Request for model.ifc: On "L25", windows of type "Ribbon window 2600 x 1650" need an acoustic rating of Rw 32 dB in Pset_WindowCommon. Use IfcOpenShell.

First a look at what the model holds.

```python
import ifcopenshell
import ifcopenshell.util.element

model = ifcopenshell.open("model.ifc")
print(model.schema)
storey = next(s for s in model.by_type("IfcBuildingStorey") if s.Name == "L25")
windows = [e for e in ifcopenshell.util.element.get_decomposition(storey) if e.is_a("IfcWindow")]
seen = {}
for e in windows:
    element_type = ifcopenshell.util.element.get_type(e)
    key = (element_type.Name if element_type != e and element_type else None, ifcopenshell.util.element.get_pset(e, "Pset_WindowCommon", "AcousticRating"))
    seen[key] = seen.get(key, 0) + 1
for (name, value), count in sorted(seen.items(), key=str):
    print(count, "x", name, "|", value)
```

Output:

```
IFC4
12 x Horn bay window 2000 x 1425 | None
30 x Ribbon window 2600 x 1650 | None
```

```python
import ifcopenshell
import ifcopenshell.api.pset
import ifcopenshell.util.element

model = ifcopenshell.open("model.ifc")

storey = next(s for s in model.by_type("IfcBuildingStorey") if s.Name == "L25")
windows = [e for e in ifcopenshell.util.element.get_decomposition(storey) if e.is_a("IfcWindow")]

count = 0
for e in windows:
    element_type = ifcopenshell.util.element.get_type(e)
    if element_type in (None, e) or element_type.Name != "Ribbon window 2600 x 1650":
        continue
    found = ifcopenshell.util.element.get_pset(e, "Pset_WindowCommon", should_inherit=False)
    if found:
        pset = model.by_id(found["id"])
        if len(ifcopenshell.util.element.get_elements_by_pset(pset)) > 1:
            pset = ifcopenshell.api.pset.unshare_pset(model, products=[e], pset=pset)[0]
    else:
        pset = ifcopenshell.api.pset.add_pset(model, product=e, name="Pset_WindowCommon")
    ifcopenshell.api.pset.edit_pset(model, pset=pset, properties={"AcousticRating": "Rw 32 dB"})
    count += 1

print(count, "windows updated")

model.write("model_rev.ifc")
```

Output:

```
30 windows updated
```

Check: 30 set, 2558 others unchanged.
